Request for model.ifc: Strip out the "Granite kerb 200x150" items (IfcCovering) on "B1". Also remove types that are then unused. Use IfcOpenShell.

First a look at what the model holds.

```python
import ifcopenshell
import ifcopenshell.util.element

model = ifcopenshell.open("model.ifc")
print(model.schema)
storey = next(s for s in model.by_type("IfcBuildingStorey") if s.Name == "B1")
coverings = [e for e in ifcopenshell.util.element.get_decomposition(storey) if e.is_a("IfcCovering")]
seen = {}
for e in coverings:
    element_type = ifcopenshell.util.element.get_type(e)
    name = element_type.Name if element_type not in (None, e) else None
    seen[name] = seen.get(name, 0) + 1
for name, count in sorted(seen.items(), key=str):
    print(count, "x", name)
```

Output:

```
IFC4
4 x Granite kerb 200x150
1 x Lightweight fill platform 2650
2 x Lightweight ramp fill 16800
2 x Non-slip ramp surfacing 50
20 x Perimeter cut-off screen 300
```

```python
import ifcopenshell
import ifcopenshell.api.root
import ifcopenshell.util.element

model = ifcopenshell.open("model.ifc")

storey = next(s for s in model.by_type("IfcBuildingStorey") if s.Name == "B1")
coverings = [e for e in ifcopenshell.util.element.get_decomposition(storey) if e.is_a("IfcCovering")]
targets = [e for e in coverings if (t := ifcopenshell.util.element.get_type(e)) not in (None, e) and t.Name == "Granite kerb 200x150"]
types = {ifcopenshell.util.element.get_type(e) for e in targets} - {None, *targets}

for e in targets:
    ifcopenshell.api.root.remove_product(model, product=e)
print(len(targets), "removed")

unused = [t for t in types if not ifcopenshell.util.element.get_types(t)]
for t in unused:
    ifcopenshell.api.root.remove_product(model, product=t)
print(len(unused), "unused types removed")

model.write("model_v2.ifc")
```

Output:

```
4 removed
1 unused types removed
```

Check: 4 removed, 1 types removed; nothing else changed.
